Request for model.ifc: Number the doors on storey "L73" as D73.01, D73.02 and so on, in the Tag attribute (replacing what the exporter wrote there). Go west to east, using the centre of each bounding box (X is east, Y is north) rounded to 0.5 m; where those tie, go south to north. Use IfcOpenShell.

First a look at what the model holds.

```python
import ifcopenshell
import ifcopenshell.util.element
import ifcopenshell.util.placement

model = ifcopenshell.open("model.ifc")
print(model.schema)
storey = next(s for s in model.by_type("IfcBuildingStorey") if s.Name == "L73")
doors = [e for e in ifcopenshell.util.element.get_decomposition(storey) if e.is_a("IfcDoor")]
for e in sorted(doors, key=lambda e: e.id()):
    origin = ifcopenshell.util.placement.get_local_placement(e.ObjectPlacement)[:3, 3]
    print(e.id(), e.Tag, e.Name, origin.round(2) + 0.0, sep=" | ")
```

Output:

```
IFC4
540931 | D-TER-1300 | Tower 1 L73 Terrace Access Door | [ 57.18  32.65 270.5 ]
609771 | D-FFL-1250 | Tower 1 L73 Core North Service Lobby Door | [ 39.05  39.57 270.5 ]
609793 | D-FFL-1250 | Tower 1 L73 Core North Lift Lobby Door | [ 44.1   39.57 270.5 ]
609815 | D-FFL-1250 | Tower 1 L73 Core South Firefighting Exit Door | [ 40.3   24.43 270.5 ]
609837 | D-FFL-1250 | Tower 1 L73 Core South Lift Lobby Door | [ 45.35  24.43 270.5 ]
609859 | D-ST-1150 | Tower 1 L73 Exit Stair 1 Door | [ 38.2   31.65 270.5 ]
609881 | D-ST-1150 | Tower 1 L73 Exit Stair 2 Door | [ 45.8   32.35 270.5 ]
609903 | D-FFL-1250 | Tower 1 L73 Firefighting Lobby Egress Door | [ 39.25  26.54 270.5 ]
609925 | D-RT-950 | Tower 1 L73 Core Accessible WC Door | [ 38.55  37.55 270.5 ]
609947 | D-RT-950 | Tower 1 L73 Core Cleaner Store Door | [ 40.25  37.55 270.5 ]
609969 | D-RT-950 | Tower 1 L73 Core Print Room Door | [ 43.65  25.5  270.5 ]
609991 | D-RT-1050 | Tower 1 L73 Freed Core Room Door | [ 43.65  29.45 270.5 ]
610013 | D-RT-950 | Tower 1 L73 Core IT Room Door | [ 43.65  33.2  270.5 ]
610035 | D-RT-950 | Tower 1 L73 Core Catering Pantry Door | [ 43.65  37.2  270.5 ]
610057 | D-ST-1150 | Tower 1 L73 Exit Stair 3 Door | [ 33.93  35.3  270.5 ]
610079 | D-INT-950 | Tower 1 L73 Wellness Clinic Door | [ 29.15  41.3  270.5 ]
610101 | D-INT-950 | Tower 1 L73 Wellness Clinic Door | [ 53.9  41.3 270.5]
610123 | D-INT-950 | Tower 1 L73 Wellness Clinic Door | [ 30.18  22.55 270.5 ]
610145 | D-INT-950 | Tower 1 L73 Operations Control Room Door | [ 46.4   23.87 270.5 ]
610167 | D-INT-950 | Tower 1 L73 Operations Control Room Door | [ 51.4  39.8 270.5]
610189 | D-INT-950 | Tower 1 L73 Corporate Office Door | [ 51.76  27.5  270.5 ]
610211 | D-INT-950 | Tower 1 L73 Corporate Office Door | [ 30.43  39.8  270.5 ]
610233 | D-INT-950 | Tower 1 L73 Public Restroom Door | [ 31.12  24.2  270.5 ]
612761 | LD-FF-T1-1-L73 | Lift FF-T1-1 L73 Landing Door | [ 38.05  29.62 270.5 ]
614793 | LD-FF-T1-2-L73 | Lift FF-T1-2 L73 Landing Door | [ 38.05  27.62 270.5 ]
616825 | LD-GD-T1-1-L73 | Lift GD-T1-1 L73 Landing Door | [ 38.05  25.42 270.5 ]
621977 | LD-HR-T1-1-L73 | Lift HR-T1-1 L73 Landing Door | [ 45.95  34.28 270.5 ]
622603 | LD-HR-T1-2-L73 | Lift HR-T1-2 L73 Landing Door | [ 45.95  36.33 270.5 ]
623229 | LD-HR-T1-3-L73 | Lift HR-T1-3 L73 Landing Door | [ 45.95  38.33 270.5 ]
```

```python
import ifcopenshell
import ifcopenshell.geom
import ifcopenshell.util.element
import ifcopenshell.util.shape

model = ifcopenshell.open("model.ifc")
settings = ifcopenshell.geom.settings()
settings.set("use-world-coords", True)


def centre(element):
    shape = ifcopenshell.geom.create_shape(settings, element)
    return ifcopenshell.util.shape.get_bbox_centroid(shape.geometry)


storey = next(s for s in model.by_type("IfcBuildingStorey") if s.Name == "L73")
doors = [e for e in ifcopenshell.util.element.get_decomposition(storey) if e.is_a("IfcDoor")]

# Insertion points can sit at a corner or the storey origin, so sort by the geometry (in metres).
centres = {e: centre(e) for e in doors}
doors.sort(key=lambda e: (round(centres[e][0] / 0.5), centres[e][1]))

for i, e in enumerate(doors, start=1):
    number = f"D73.{i:02d}"
    e.Tag = number
    print(e.id(), number)

model.write("model_rev.ifc")
```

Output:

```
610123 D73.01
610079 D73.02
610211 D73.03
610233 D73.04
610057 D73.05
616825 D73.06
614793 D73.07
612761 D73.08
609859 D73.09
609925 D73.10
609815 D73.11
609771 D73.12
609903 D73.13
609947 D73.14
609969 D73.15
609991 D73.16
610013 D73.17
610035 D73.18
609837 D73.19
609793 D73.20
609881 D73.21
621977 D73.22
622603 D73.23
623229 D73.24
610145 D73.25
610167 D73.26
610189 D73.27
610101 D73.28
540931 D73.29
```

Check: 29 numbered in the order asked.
